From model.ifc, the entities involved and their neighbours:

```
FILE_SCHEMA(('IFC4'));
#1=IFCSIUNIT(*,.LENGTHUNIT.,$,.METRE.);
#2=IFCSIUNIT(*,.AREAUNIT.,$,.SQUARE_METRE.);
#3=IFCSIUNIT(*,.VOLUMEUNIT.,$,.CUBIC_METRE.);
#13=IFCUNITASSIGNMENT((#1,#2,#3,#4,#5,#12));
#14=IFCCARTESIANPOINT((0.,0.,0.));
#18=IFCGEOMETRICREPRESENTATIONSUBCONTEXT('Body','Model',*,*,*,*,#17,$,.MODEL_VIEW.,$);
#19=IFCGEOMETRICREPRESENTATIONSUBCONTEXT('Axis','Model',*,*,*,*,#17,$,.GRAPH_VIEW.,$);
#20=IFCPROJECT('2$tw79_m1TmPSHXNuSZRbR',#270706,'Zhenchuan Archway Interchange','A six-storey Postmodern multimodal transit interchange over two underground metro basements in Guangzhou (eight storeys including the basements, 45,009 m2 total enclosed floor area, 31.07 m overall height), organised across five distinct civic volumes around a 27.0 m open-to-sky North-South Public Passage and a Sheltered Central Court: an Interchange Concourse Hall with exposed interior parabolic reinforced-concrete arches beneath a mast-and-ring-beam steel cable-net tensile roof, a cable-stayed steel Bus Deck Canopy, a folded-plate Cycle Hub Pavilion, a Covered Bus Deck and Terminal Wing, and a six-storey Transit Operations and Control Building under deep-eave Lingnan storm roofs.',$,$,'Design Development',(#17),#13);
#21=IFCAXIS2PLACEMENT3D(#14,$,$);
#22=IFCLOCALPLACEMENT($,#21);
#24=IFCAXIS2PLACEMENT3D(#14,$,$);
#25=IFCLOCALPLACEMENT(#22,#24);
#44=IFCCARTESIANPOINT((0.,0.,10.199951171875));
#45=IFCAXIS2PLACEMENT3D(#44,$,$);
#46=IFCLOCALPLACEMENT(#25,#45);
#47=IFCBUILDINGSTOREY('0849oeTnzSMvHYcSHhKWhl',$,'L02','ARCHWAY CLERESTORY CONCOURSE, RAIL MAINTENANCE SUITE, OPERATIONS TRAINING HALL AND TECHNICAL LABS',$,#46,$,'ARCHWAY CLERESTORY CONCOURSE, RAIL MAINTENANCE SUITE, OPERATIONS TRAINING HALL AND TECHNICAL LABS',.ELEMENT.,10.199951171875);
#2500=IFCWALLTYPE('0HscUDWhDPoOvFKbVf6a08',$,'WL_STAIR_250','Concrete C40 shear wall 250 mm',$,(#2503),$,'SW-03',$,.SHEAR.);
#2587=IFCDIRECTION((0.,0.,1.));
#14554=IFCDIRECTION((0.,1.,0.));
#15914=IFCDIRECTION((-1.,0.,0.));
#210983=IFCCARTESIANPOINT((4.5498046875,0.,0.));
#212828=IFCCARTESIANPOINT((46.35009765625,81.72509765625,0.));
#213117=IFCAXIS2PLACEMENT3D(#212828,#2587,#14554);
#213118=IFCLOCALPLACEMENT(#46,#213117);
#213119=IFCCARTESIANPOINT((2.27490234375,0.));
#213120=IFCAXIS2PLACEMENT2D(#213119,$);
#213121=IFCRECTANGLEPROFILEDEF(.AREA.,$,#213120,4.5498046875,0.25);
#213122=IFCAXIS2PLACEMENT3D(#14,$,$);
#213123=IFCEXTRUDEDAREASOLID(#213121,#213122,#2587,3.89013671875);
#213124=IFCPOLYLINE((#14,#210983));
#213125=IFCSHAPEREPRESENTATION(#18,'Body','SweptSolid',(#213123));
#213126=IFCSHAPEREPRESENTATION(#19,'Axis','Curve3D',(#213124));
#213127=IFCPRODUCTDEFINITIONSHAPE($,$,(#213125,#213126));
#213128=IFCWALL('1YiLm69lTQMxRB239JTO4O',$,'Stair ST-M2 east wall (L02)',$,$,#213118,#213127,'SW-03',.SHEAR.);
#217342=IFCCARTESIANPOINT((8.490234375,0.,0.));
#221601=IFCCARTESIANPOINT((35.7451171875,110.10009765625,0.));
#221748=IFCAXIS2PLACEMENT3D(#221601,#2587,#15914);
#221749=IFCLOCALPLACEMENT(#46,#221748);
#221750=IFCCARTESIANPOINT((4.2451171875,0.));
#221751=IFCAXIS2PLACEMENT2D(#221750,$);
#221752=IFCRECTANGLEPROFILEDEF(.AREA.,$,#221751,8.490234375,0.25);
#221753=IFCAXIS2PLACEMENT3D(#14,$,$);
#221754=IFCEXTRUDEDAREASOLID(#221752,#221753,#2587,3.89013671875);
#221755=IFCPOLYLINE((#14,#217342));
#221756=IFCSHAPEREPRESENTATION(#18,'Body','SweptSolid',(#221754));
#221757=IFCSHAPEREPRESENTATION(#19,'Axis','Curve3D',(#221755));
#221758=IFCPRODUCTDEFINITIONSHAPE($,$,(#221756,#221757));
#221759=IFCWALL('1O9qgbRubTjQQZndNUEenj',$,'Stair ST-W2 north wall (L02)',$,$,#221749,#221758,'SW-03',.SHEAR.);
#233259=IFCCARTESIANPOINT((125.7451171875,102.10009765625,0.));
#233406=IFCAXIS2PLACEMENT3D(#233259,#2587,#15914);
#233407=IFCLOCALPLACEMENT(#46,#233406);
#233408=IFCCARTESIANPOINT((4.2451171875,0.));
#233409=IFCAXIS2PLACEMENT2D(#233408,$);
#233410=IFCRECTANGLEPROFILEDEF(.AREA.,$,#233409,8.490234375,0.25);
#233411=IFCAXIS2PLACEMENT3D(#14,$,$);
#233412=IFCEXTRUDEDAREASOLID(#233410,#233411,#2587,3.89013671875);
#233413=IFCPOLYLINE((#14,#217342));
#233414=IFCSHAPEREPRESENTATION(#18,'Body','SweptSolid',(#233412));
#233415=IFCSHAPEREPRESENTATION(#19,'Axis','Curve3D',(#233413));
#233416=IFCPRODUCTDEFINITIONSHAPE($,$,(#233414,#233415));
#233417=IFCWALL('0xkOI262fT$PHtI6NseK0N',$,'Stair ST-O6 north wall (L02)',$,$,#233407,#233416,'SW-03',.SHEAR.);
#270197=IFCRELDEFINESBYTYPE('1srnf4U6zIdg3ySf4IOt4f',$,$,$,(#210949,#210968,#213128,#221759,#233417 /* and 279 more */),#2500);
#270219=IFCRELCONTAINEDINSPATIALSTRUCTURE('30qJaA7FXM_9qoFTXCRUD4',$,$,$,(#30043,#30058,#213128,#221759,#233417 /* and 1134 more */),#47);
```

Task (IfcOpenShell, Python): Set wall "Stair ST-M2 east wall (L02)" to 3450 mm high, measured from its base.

```python
import ifcopenshell
import ifcopenshell.geom
import ifcopenshell.util.representation
import ifcopenshell.util.shape
import ifcopenshell.util.unit

model = ifcopenshell.open("model.ifc")
unit_scale = ifcopenshell.util.unit.calculate_unit_scale(model)
settings = ifcopenshell.geom.settings()


def volume(element):
    """Net volume in cubic metres, openings subtracted."""
    shape = ifcopenshell.geom.create_shape(settings, element)
    return ifcopenshell.util.shape.get_volume(shape.geometry)


wall = model.by_guid("1YiLm69lTQMxRB239JTO4O")
before = volume(wall)

body = ifcopenshell.util.representation.get_representation(wall, "Model", "Body")
solid = body.Items[0]
old_height = solid.Depth
solid.Depth = 3.45 / unit_scale
after = volume(wall)

print(f"height {old_height:g} -> {solid.Depth:g}, volume {before:.3f} -> {after:.3f} m3")

model.write("model-out.ifc")
```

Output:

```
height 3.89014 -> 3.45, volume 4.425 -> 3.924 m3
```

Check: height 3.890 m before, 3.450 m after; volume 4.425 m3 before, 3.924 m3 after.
